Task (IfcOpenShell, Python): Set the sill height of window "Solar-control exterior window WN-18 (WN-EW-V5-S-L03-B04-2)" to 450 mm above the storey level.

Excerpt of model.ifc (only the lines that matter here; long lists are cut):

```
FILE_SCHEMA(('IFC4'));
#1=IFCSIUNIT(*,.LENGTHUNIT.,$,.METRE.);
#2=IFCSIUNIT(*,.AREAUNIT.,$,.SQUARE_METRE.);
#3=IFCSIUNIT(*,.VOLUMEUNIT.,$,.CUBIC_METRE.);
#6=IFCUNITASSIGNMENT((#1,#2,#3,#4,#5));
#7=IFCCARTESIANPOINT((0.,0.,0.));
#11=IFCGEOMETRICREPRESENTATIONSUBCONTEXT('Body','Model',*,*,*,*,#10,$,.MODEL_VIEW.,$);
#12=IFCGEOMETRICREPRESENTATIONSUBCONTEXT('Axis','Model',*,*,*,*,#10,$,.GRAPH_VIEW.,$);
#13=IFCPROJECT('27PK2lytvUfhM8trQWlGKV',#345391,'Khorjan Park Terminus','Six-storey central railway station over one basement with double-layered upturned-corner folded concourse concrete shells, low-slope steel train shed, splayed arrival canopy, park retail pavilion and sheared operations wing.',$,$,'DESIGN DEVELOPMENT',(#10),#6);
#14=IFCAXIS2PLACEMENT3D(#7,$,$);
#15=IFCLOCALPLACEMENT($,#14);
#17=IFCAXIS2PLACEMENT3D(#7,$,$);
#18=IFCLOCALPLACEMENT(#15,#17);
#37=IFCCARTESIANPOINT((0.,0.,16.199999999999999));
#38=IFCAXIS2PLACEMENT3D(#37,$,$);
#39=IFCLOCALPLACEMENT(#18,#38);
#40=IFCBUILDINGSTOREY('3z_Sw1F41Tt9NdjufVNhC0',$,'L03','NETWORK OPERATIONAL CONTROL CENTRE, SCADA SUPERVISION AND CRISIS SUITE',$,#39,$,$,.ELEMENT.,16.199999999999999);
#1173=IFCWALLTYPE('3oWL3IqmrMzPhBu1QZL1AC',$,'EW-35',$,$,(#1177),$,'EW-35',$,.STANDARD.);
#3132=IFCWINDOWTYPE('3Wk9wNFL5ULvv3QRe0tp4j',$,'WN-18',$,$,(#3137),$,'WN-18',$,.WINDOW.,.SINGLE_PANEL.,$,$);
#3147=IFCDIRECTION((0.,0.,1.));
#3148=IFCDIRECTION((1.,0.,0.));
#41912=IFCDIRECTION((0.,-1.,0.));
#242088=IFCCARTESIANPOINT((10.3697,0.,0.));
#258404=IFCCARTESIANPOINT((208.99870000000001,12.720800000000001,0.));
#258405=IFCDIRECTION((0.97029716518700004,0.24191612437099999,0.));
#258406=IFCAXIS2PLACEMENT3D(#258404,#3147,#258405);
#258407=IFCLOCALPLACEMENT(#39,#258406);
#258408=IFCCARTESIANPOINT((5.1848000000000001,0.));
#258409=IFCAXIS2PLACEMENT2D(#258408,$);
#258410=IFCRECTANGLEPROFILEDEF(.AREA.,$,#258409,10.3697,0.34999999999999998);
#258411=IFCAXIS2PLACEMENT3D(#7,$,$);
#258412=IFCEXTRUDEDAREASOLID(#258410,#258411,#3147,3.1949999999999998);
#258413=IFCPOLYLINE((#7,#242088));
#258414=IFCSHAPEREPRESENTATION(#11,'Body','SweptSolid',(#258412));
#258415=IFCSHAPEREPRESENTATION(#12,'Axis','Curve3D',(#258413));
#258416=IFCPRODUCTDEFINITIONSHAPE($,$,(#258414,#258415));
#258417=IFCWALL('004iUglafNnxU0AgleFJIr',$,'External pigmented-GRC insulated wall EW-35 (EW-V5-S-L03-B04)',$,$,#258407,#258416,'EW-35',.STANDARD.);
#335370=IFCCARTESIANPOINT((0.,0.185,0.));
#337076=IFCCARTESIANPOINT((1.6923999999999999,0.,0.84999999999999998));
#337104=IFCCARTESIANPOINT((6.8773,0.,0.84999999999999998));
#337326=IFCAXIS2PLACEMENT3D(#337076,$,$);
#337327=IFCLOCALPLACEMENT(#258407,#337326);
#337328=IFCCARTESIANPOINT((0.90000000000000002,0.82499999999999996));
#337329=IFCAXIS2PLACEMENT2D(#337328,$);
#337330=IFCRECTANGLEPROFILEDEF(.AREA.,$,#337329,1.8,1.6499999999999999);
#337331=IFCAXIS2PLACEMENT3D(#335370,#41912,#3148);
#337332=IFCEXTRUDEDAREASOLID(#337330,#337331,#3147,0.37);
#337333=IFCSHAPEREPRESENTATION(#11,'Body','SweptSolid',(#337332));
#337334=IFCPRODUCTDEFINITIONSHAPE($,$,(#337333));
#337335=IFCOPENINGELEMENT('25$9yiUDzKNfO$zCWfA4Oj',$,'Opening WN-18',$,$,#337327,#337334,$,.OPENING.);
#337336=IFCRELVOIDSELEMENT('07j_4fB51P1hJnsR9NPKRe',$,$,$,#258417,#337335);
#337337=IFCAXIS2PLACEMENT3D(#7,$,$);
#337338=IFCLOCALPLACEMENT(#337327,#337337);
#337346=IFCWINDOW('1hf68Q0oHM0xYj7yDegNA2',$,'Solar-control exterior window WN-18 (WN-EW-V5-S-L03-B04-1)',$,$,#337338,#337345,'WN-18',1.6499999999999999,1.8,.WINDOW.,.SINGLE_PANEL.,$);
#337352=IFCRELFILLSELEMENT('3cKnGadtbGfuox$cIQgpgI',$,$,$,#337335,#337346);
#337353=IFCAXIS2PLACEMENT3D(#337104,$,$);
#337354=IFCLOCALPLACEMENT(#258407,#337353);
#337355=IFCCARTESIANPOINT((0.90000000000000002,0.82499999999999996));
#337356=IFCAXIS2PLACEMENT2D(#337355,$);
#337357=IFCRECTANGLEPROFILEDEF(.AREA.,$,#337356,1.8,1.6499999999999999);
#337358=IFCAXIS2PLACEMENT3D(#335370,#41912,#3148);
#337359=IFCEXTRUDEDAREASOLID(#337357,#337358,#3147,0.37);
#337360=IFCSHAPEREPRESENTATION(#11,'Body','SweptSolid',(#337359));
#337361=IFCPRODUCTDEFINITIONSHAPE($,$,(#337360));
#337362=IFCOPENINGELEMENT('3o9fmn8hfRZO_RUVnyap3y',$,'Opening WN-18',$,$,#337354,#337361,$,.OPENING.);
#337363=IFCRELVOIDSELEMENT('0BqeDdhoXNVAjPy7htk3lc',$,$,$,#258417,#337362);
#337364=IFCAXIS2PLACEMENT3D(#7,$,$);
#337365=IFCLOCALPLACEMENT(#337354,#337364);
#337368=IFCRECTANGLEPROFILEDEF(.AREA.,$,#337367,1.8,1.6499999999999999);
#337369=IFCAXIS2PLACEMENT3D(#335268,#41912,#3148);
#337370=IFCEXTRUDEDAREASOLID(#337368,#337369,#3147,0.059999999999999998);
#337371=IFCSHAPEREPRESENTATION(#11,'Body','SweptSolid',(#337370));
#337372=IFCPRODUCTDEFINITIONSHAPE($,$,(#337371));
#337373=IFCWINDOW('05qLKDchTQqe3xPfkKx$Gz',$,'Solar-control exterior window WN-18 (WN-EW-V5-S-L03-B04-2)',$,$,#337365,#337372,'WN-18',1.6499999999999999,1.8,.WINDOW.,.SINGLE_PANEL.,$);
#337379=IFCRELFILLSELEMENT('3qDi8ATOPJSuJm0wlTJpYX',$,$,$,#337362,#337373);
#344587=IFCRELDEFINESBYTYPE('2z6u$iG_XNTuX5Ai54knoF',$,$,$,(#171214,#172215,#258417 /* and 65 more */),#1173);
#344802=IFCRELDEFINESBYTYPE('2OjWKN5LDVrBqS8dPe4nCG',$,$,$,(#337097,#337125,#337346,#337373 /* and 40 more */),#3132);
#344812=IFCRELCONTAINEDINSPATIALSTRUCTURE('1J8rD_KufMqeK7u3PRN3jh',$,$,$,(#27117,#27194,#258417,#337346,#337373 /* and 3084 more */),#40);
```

```python
import numpy as np
import ifcopenshell
import ifcopenshell.api.geometry
import ifcopenshell.geom
import ifcopenshell.util.element
import ifcopenshell.util.placement
import ifcopenshell.util.shape
import ifcopenshell.util.unit

model = ifcopenshell.open("model.ifc")
unit_scale = ifcopenshell.util.unit.calculate_unit_scale(model)

window = model.by_id(337373)
opening = window.FillsVoids[0].RelatingOpeningElement
storey = ifcopenshell.util.element.get_container(window, ifc_class="IfcBuildingStorey")
level = ifcopenshell.util.placement.get_local_placement(storey.ObjectPlacement)[2, 3]

# The opening's origin need not be at the sill, so measure its lowest point.
shape = ifcopenshell.geom.create_shape(ifcopenshell.geom.settings(), opening)
bottom = ifcopenshell.util.shape.get_shape_bottom_elevation(shape, shape.geometry) / unit_scale
dz = level + 0.45 / unit_scale - bottom

shift = np.array([0.0, 0.0, dz])
# The window is placed relative to its opening, so it follows when the opening moves.
matrix = ifcopenshell.util.placement.get_local_placement(opening.ObjectPlacement)
matrix[:3, 3] += shift
ifcopenshell.api.geometry.edit_object_placement(
    model, product=opening, matrix=matrix, is_si=False, should_transform_children=True
)

print(f"moved by {dz * unit_scale:+.3f} m")

model.write("model_edited.ifc")
```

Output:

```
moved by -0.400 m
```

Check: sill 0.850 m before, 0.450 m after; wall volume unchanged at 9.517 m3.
